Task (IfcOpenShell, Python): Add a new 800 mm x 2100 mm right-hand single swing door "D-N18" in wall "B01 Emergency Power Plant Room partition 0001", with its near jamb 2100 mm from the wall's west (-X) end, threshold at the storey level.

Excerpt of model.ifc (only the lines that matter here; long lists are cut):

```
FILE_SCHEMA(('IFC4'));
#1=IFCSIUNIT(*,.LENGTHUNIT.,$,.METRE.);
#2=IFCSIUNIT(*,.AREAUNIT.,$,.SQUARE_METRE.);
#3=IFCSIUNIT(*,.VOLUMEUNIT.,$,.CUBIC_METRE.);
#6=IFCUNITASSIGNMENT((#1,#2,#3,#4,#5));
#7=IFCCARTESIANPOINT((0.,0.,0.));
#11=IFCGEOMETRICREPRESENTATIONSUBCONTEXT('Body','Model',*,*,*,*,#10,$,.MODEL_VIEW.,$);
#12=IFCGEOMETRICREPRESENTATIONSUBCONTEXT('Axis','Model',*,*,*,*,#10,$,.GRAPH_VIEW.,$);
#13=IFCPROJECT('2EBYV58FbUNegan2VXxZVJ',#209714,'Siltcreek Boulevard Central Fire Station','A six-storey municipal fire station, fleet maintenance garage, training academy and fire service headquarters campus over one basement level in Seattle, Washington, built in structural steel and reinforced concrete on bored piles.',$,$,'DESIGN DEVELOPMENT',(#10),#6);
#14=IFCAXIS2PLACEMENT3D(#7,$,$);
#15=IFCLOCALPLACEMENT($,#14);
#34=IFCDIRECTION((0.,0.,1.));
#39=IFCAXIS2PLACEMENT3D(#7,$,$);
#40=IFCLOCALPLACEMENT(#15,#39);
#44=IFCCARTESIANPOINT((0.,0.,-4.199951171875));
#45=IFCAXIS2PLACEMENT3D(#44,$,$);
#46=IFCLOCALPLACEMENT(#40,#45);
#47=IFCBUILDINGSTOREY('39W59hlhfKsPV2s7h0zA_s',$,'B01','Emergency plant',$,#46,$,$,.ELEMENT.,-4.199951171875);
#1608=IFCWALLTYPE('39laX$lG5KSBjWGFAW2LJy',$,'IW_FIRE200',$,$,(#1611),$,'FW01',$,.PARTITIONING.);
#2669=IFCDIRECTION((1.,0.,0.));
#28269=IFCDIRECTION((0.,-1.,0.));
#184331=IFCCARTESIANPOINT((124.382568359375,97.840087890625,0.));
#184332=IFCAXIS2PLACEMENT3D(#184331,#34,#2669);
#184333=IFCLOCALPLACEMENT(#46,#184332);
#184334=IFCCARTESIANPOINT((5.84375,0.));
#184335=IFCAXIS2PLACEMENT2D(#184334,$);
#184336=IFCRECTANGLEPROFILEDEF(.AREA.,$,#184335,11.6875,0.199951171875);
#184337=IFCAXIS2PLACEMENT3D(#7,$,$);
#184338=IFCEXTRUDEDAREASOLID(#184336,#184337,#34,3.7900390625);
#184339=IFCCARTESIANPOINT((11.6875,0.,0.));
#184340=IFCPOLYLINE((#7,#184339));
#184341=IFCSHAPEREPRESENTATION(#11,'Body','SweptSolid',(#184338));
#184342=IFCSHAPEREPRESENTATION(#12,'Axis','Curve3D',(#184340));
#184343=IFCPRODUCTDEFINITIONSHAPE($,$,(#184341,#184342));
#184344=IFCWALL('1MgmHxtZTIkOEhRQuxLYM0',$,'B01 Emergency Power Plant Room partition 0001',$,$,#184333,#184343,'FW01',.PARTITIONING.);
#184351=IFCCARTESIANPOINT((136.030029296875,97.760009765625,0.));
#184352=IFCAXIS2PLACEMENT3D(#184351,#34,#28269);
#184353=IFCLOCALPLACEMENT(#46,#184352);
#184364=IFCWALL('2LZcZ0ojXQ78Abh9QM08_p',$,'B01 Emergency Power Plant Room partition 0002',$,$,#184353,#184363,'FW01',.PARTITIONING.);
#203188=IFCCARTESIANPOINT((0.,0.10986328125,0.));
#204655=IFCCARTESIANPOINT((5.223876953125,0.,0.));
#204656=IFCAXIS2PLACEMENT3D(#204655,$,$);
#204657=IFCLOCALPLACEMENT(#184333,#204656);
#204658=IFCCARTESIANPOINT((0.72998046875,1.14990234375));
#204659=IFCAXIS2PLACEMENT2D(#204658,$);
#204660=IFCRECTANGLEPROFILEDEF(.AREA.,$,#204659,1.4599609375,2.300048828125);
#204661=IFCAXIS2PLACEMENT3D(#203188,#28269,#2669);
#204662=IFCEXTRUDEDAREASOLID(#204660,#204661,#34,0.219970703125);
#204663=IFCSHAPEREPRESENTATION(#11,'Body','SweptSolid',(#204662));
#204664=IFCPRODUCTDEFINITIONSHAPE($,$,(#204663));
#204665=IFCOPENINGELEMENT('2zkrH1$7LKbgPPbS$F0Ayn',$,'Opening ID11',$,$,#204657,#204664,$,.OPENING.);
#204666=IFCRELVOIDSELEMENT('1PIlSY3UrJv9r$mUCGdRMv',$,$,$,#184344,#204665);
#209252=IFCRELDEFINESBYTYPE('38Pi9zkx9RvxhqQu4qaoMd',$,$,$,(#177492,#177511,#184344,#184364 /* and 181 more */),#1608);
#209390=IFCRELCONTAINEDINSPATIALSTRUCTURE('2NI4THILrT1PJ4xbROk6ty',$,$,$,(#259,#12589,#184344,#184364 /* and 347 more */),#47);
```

```python
import numpy as np
import ifcopenshell
import ifcopenshell.api.feature
import ifcopenshell.api.geometry
import ifcopenshell.api.root
import ifcopenshell.api.spatial
import ifcopenshell.geom
import ifcopenshell.util.element
import ifcopenshell.util.placement
import ifcopenshell.util.representation
import ifcopenshell.util.shape
import ifcopenshell.util.unit

model = ifcopenshell.open("model.ifc")
unit_scale = ifcopenshell.util.unit.calculate_unit_scale(model)
settings = ifcopenshell.geom.settings()


def volume(element):
    """Net volume in cubic metres, openings subtracted."""
    shape = ifcopenshell.geom.create_shape(settings, element)
    return ifcopenshell.util.shape.get_volume(shape.geometry)


wall = model.by_guid("1MgmHxtZTIkOEhRQuxLYM0")
storey = ifcopenshell.util.element.get_container(wall, ifc_class="IfcBuildingStorey")
context = ifcopenshell.util.representation.get_context(model, "Model", "Body", "MODEL_VIEW")
before = volume(wall)

width, height, from_end, sill = 0.8, 2.1, 2.1, 0.0  # metres

# The wall runs along its own X axis, and the end named is its -X end.
wall_shape = ifcopenshell.geom.create_shape(settings, wall)
x, y, z = ifcopenshell.util.shape.get_vertices(wall_shape.geometry).T
start = x.min() + from_end
face, thickness = float(y.min()), float(y.max() - y.min())
wall_matrix = ifcopenshell.util.placement.get_local_placement(wall.ObjectPlacement)
level = ifcopenshell.util.placement.get_local_placement(storey.ObjectPlacement)[2, 3]


def in_wall(x, y):
    """Placement at x, y metres in the wall's axes, at sill height."""
    matrix = wall_matrix.copy()
    matrix[:, 3] = wall_matrix @ np.array([x / unit_scale, y / unit_scale, 0.0, 1.0])
    matrix[2, 3] = level + sill / unit_scale
    return matrix


# Opening: a box that overshoots both wall faces by 50 mm.
opening = ifcopenshell.api.root.create_entity(model, ifc_class="IfcOpeningElement", predefined_type="OPENING")
box = ifcopenshell.api.geometry.add_wall_representation(
    model, context=context, length=width, height=height, thickness=thickness + 0.1
)
ifcopenshell.api.geometry.assign_representation(model, product=opening, representation=box)
ifcopenshell.api.geometry.edit_object_placement(model, product=opening, matrix=in_wall(start, face - 0.05), is_si=False)
ifcopenshell.api.feature.add_feature(model, feature=opening, element=wall)

door = ifcopenshell.api.root.create_entity(model, ifc_class="IfcDoor", name="D-N18", predefined_type="DOOR")
door.OverallWidth, door.OverallHeight = width / unit_scale, height / unit_scale
door.OperationType = "SINGLE_SWING_RIGHT"
body = ifcopenshell.api.geometry.add_door_representation(
    model,
    context=context,
    overall_width=door.OverallWidth,
    overall_height=door.OverallHeight,
    operation_type="SINGLE_SWING_RIGHT",
    lining_properties={"LiningDepth": thickness / unit_scale, "ThresholdDepth": thickness / unit_scale},
)
ifcopenshell.api.geometry.assign_representation(model, product=door, representation=body)
ifcopenshell.api.spatial.assign_container(model, products=[door], relating_structure=storey)
ifcopenshell.api.feature.add_filling(model, opening=opening, element=door)

# The lining spans the wall, so the door starts at the wall face.
ifcopenshell.api.geometry.edit_object_placement(model, product=door, matrix=in_wall(start, face), is_si=False)

after = volume(wall)

print(f"wall volume {before:.3f} -> {after:.3f} m3")

model.write("model_rev.ifc")
```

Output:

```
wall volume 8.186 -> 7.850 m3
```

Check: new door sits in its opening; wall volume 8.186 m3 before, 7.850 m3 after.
